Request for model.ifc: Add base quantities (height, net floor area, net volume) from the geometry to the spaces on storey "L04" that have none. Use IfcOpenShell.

First a look at what the model holds.

```python
import ifcopenshell
import ifcopenshell.util.element
import ifcopenshell.util.unit

model = ifcopenshell.open("model.ifc")
print(model.schema)
for unit_type in ("LENGTHUNIT", "AREAUNIT", "VOLUMEUNIT"):
    print(unit_type, ifcopenshell.util.unit.calculate_unit_scale(model, unit_type))
storey = next(s for s in model.by_type("IfcBuildingStorey") if s.Name == "L04")
spaces = [e for e in ifcopenshell.util.element.get_decomposition(storey) if e.is_a("IfcSpace")]
for e in sorted(spaces, key=lambda e: e.id()):
    print(e.id(), e.is_a(), e.Name, list(ifcopenshell.util.element.get_psets(e, qtos_only=True)), sep=" | ")
```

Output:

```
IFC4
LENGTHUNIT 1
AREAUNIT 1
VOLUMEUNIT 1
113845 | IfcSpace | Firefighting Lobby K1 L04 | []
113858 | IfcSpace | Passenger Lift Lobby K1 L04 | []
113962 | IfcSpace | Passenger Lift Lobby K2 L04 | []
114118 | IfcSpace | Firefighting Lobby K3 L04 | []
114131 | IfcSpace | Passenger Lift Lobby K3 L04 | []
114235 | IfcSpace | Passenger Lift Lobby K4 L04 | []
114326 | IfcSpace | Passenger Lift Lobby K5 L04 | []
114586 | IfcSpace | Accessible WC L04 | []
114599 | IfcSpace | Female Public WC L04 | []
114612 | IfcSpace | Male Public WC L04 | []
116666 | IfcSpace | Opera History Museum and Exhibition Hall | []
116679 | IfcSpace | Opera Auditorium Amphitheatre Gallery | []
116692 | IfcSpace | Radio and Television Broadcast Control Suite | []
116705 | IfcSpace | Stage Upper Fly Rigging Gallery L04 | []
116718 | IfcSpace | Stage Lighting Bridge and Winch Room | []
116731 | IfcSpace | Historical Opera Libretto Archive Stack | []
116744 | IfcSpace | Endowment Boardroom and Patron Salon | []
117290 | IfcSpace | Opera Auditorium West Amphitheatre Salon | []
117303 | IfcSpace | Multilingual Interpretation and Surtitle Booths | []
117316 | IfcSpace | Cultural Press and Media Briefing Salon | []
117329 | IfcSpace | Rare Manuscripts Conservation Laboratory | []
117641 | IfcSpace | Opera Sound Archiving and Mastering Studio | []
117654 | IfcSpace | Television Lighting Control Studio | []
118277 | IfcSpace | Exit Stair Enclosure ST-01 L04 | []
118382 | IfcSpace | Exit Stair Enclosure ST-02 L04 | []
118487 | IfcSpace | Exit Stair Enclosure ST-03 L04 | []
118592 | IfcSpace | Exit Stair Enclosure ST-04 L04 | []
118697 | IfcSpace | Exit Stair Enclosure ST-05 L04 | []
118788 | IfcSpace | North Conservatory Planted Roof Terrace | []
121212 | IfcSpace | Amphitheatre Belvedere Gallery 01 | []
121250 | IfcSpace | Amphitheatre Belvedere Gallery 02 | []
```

```python
import ifcopenshell
import ifcopenshell.api.pset
import ifcopenshell.geom
import ifcopenshell.util.element
import ifcopenshell.util.shape
import ifcopenshell.util.unit

model = ifcopenshell.open("model.ifc")
unit_scale = ifcopenshell.util.unit.calculate_unit_scale(model)
area_scale = ifcopenshell.util.unit.calculate_unit_scale(model, "AREAUNIT")
volume_scale = ifcopenshell.util.unit.calculate_unit_scale(model, "VOLUMEUNIT")
settings = ifcopenshell.geom.settings()

storey = next(s for s in model.by_type("IfcBuildingStorey") if s.Name == "L04")
spaces = [e for e in ifcopenshell.util.element.get_decomposition(storey) if e.is_a("IfcSpace")]

for e in sorted(spaces, key=lambda e: e.id()):
    if ifcopenshell.util.element.get_psets(e, qtos_only=True, should_inherit=False):
        continue
    # Geometry comes back in metres, in the element's own axes.
    shape = ifcopenshell.geom.create_shape(settings, e)
    values = {
        "Height": ifcopenshell.util.shape.get_z(shape.geometry) / unit_scale,
        "NetFloorArea": ifcopenshell.util.shape.get_footprint_area(shape.geometry) / area_scale,
        "NetVolume": ifcopenshell.util.shape.get_volume(shape.geometry) / volume_scale,
    }
    qto = ifcopenshell.api.pset.add_qto(model, product=e, name="Qto_SpaceBaseQuantities")
    ifcopenshell.api.pset.edit_qto(model, qto=qto, properties=values)
    print(e.id(), {k: round(v, 3) for k, v in values.items()})

model.write("model_v2.ifc")
```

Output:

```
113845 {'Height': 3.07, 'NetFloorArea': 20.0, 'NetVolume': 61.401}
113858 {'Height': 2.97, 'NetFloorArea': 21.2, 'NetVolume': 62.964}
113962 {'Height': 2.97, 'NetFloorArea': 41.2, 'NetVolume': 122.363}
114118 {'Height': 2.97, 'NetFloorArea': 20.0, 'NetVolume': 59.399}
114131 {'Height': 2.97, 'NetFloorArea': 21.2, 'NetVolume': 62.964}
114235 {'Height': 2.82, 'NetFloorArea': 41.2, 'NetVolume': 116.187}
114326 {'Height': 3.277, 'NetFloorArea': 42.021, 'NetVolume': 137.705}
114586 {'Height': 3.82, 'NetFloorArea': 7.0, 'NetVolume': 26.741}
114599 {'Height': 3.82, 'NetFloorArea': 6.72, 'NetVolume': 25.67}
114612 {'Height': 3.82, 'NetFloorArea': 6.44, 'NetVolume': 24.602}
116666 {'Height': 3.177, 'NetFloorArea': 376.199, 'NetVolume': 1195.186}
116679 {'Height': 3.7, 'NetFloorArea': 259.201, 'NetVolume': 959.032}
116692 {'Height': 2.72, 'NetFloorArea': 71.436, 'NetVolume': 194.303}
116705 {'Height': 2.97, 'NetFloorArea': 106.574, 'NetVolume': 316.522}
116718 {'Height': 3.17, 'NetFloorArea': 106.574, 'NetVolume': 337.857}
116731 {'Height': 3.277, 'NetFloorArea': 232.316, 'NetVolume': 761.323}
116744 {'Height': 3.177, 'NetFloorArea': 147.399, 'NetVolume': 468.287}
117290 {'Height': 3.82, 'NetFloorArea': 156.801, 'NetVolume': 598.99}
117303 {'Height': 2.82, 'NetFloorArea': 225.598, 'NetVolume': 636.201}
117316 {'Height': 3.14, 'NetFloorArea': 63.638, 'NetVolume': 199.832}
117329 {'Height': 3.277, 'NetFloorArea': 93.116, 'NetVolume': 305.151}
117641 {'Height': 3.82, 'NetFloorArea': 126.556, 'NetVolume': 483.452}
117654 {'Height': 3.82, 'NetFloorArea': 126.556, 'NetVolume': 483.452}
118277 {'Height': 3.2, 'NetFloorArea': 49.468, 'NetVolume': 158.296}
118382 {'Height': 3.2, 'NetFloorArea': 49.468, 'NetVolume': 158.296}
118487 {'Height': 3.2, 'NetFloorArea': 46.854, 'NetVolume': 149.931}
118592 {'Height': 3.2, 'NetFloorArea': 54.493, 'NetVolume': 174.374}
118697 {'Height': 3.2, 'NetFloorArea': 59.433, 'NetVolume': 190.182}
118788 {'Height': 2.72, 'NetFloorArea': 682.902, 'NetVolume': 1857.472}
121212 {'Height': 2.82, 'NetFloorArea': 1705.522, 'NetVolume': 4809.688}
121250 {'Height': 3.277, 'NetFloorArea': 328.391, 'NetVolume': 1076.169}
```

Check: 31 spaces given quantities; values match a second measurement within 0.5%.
